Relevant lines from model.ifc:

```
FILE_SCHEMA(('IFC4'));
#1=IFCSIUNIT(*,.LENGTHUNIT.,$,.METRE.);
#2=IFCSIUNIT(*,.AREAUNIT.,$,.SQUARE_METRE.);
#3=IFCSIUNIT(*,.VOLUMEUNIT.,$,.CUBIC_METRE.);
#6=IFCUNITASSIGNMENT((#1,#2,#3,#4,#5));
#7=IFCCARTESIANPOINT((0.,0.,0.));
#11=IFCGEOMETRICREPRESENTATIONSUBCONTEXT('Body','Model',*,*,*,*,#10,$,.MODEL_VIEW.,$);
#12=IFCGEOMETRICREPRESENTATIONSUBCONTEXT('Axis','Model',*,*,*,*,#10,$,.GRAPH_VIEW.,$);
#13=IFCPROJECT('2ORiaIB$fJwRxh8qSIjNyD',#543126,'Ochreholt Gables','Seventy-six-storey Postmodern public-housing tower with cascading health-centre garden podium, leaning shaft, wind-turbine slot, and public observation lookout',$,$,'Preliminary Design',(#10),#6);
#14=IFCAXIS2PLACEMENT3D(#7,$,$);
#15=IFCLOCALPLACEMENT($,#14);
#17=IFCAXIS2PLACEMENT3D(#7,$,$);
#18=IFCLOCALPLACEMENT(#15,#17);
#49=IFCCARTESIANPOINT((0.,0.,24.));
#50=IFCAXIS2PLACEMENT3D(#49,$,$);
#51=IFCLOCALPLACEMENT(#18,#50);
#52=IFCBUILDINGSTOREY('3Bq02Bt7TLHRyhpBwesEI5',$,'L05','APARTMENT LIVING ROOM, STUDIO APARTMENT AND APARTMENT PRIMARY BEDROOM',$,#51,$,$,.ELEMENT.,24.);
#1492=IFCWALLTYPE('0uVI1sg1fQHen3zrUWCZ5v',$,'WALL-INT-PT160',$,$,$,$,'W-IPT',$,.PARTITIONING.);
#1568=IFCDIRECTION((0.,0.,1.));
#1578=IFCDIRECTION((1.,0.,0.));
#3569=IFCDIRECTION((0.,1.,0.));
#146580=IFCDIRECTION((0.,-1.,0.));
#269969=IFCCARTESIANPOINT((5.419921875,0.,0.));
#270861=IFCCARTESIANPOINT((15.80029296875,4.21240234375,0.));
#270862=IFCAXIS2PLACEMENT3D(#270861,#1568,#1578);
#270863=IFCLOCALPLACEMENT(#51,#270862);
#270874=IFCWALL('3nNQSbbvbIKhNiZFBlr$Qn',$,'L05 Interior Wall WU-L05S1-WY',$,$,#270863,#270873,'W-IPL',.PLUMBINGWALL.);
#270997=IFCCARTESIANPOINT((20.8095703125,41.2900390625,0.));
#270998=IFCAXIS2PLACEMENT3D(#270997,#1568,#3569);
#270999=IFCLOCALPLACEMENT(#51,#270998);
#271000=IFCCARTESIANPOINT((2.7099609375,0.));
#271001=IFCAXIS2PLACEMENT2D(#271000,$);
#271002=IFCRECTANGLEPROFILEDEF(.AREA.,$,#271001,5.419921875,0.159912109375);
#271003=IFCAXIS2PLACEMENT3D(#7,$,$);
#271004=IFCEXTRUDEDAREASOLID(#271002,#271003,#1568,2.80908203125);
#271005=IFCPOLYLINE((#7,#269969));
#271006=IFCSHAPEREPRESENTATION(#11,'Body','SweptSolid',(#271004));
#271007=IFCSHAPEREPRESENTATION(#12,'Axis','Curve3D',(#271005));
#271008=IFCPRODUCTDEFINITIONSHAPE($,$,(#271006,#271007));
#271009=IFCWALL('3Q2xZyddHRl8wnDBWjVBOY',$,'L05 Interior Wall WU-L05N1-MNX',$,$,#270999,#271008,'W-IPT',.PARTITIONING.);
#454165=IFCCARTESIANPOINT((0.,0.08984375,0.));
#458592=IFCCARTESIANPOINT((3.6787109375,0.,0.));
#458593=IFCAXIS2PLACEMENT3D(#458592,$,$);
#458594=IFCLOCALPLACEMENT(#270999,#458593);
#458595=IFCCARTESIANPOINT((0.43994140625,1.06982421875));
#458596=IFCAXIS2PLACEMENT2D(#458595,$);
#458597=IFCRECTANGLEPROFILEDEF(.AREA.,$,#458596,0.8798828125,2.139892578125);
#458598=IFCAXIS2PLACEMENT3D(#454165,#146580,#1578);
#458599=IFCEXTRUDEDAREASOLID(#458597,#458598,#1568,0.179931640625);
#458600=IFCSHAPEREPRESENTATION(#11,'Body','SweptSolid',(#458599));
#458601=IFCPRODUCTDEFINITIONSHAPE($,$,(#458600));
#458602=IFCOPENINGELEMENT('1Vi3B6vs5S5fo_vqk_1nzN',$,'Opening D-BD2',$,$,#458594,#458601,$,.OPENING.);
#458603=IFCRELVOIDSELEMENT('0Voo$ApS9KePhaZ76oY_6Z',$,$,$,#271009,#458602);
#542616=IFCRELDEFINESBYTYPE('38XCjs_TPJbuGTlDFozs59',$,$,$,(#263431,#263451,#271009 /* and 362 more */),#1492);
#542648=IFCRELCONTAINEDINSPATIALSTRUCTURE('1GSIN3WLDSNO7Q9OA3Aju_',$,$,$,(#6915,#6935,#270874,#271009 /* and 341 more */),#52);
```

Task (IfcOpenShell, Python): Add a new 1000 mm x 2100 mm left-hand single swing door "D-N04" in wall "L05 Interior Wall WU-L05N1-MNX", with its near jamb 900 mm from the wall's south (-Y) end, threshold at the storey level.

```python
import numpy as np
import ifcopenshell
import ifcopenshell.api.feature
import ifcopenshell.api.geometry
import ifcopenshell.api.root
import ifcopenshell.api.spatial
import ifcopenshell.geom
import ifcopenshell.util.element
import ifcopenshell.util.placement
import ifcopenshell.util.representation
import ifcopenshell.util.shape
import ifcopenshell.util.unit

model = ifcopenshell.open("model.ifc")
unit_scale = ifcopenshell.util.unit.calculate_unit_scale(model)
settings = ifcopenshell.geom.settings()


def volume(element):
    """Net volume in cubic metres, openings subtracted."""
    shape = ifcopenshell.geom.create_shape(settings, element)
    return ifcopenshell.util.shape.get_volume(shape.geometry)


wall = model.by_guid("3Q2xZyddHRl8wnDBWjVBOY")
storey = ifcopenshell.util.element.get_container(wall, ifc_class="IfcBuildingStorey")
context = ifcopenshell.util.representation.get_context(model, "Model", "Body", "MODEL_VIEW")
before = volume(wall)

width, height, from_end, sill = 1, 2.1, 0.9, 0.0  # metres

# The wall runs along its own X axis, and the end named is its -X end.
wall_shape = ifcopenshell.geom.create_shape(settings, wall)
x, y, z = ifcopenshell.util.shape.get_vertices(wall_shape.geometry).T
start = x.min() + from_end
face, thickness = float(y.min()), float(y.max() - y.min())
wall_matrix = ifcopenshell.util.placement.get_local_placement(wall.ObjectPlacement)
level = ifcopenshell.util.placement.get_local_placement(storey.ObjectPlacement)[2, 3]


def in_wall(x, y):
    """Placement at x, y metres in the wall's axes, at sill height."""
    matrix = wall_matrix.copy()
    matrix[:, 3] = wall_matrix @ np.array([x / unit_scale, y / unit_scale, 0.0, 1.0])
    matrix[2, 3] = level + sill / unit_scale
    return matrix


# Opening: a box that overshoots both wall faces by 50 mm.
opening = ifcopenshell.api.root.create_entity(model, ifc_class="IfcOpeningElement", predefined_type="OPENING")
box = ifcopenshell.api.geometry.add_wall_representation(
    model, context=context, length=width, height=height, thickness=thickness + 0.1
)
ifcopenshell.api.geometry.assign_representation(model, product=opening, representation=box)
ifcopenshell.api.geometry.edit_object_placement(model, product=opening, matrix=in_wall(start, face - 0.05), is_si=False)
ifcopenshell.api.feature.add_feature(model, feature=opening, element=wall)

door = ifcopenshell.api.root.create_entity(model, ifc_class="IfcDoor", name="D-N04", predefined_type="DOOR")
door.OverallWidth, door.OverallHeight = width / unit_scale, height / unit_scale
door.OperationType = "SINGLE_SWING_LEFT"
body = ifcopenshell.api.geometry.add_door_representation(
    model,
    context=context,
    overall_width=door.OverallWidth,
    overall_height=door.OverallHeight,
    operation_type="SINGLE_SWING_LEFT",
    lining_properties={"LiningDepth": thickness / unit_scale, "ThresholdDepth": thickness / unit_scale},
)
ifcopenshell.api.geometry.assign_representation(model, product=door, representation=body)
ifcopenshell.api.spatial.assign_container(model, products=[door], relating_structure=storey)
ifcopenshell.api.feature.add_filling(model, opening=opening, element=door)

# The lining spans the wall, so the door starts at the wall face.
ifcopenshell.api.geometry.edit_object_placement(model, product=door, matrix=in_wall(start, face), is_si=False)

after = volume(wall)

print(f"wall volume {before:.3f} -> {after:.3f} m3")

model.write("model_updated.ifc")
```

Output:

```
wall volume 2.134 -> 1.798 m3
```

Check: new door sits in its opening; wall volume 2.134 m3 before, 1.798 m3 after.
